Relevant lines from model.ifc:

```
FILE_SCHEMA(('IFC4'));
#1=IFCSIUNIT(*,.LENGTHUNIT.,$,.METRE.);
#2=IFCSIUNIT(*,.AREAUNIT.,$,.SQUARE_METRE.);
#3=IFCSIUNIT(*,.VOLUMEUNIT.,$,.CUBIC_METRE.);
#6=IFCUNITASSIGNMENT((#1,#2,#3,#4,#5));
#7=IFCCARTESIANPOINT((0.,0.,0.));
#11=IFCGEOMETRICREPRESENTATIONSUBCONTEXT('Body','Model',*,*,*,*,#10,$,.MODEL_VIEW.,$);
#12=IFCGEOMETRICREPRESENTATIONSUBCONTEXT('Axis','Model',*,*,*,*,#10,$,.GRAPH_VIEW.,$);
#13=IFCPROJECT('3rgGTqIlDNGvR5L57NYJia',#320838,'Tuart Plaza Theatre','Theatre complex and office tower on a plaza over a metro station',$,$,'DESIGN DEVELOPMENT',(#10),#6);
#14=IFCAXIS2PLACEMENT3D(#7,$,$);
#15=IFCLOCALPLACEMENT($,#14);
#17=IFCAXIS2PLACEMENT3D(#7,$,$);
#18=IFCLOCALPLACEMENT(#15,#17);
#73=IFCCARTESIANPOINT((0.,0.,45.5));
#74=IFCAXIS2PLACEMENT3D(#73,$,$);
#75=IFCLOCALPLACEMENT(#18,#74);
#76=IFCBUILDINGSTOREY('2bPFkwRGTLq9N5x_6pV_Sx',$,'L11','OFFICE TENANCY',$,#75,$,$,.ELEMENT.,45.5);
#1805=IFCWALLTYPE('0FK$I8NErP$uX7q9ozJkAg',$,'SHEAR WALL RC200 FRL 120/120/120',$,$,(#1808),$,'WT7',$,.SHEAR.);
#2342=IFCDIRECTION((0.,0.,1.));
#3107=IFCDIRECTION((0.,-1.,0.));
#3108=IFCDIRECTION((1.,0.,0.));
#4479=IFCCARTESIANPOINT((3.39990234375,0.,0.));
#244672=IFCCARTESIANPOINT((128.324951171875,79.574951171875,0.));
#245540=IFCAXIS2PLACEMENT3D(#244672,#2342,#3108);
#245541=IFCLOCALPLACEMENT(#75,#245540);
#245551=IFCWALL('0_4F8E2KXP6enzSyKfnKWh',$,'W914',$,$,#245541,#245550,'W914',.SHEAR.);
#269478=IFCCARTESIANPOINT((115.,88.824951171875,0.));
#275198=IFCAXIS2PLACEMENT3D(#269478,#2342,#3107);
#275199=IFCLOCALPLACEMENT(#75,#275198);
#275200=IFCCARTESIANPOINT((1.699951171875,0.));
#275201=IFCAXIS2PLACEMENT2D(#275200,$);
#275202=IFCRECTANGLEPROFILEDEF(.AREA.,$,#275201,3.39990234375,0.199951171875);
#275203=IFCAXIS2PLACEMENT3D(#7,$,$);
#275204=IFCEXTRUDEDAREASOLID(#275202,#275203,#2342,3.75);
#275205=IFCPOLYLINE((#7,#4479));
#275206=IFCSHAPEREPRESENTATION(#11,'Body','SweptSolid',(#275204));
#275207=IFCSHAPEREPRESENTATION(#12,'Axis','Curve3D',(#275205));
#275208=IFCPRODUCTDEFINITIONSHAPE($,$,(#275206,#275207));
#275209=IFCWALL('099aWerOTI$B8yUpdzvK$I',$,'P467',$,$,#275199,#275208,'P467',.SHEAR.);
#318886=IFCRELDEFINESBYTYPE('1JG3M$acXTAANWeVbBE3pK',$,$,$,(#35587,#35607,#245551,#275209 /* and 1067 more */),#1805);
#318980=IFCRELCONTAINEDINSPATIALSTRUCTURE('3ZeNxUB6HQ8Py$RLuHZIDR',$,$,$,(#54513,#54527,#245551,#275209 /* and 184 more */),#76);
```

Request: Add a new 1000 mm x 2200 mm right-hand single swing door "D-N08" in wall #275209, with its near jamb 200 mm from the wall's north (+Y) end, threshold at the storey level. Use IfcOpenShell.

```python
import numpy as np
import ifcopenshell
import ifcopenshell.api.feature
import ifcopenshell.api.geometry
import ifcopenshell.api.root
import ifcopenshell.api.spatial
import ifcopenshell.geom
import ifcopenshell.util.element
import ifcopenshell.util.placement
import ifcopenshell.util.representation
import ifcopenshell.util.shape
import ifcopenshell.util.unit

model = ifcopenshell.open("model.ifc")
unit_scale = ifcopenshell.util.unit.calculate_unit_scale(model)
settings = ifcopenshell.geom.settings()


def volume(element):
    """Net volume in cubic metres, openings subtracted."""
    shape = ifcopenshell.geom.create_shape(settings, element)
    return ifcopenshell.util.shape.get_volume(shape.geometry)


wall = model.by_guid("099aWerOTI$B8yUpdzvK$I")
storey = ifcopenshell.util.element.get_container(wall, ifc_class="IfcBuildingStorey")
context = ifcopenshell.util.representation.get_context(model, "Model", "Body", "MODEL_VIEW")
before = volume(wall)

width, height, from_end, sill = 1, 2.2, 0.2, 0.0  # metres

# The wall runs along its own X axis, and the end named is its -X end.
wall_shape = ifcopenshell.geom.create_shape(settings, wall)
x, y, z = ifcopenshell.util.shape.get_vertices(wall_shape.geometry).T
start = x.min() + from_end
face, thickness = float(y.min()), float(y.max() - y.min())
wall_matrix = ifcopenshell.util.placement.get_local_placement(wall.ObjectPlacement)
level = ifcopenshell.util.placement.get_local_placement(storey.ObjectPlacement)[2, 3]


def in_wall(x, y):
    """Placement at x, y metres in the wall's axes, at sill height."""
    matrix = wall_matrix.copy()
    matrix[:, 3] = wall_matrix @ np.array([x / unit_scale, y / unit_scale, 0.0, 1.0])
    matrix[2, 3] = level + sill / unit_scale
    return matrix


# Opening: a box that overshoots both wall faces by 50 mm.
opening = ifcopenshell.api.root.create_entity(model, ifc_class="IfcOpeningElement", predefined_type="OPENING")
box = ifcopenshell.api.geometry.add_wall_representation(
    model, context=context, length=width, height=height, thickness=thickness + 0.1
)
ifcopenshell.api.geometry.assign_representation(model, product=opening, representation=box)
ifcopenshell.api.geometry.edit_object_placement(model, product=opening, matrix=in_wall(start, face - 0.05), is_si=False)
ifcopenshell.api.feature.add_feature(model, feature=opening, element=wall)

door = ifcopenshell.api.root.create_entity(model, ifc_class="IfcDoor", name="D-N08", predefined_type="DOOR")
door.OverallWidth, door.OverallHeight = width / unit_scale, height / unit_scale
door.OperationType = "SINGLE_SWING_RIGHT"
body = ifcopenshell.api.geometry.add_door_representation(
    model,
    context=context,
    overall_width=door.OverallWidth,
    overall_height=door.OverallHeight,
    operation_type="SINGLE_SWING_RIGHT",
    lining_properties={"LiningDepth": thickness / unit_scale, "ThresholdDepth": thickness / unit_scale},
)
ifcopenshell.api.geometry.assign_representation(model, product=door, representation=body)
ifcopenshell.api.spatial.assign_container(model, products=[door], relating_structure=storey)
ifcopenshell.api.feature.add_filling(model, opening=opening, element=door)

# The lining spans the wall, so the door starts at the wall face.
ifcopenshell.api.geometry.edit_object_placement(model, product=door, matrix=in_wall(start, face), is_si=False)

after = volume(wall)

print(f"wall volume {before:.3f} -> {after:.3f} m3")

model.write("model-out.ifc")
```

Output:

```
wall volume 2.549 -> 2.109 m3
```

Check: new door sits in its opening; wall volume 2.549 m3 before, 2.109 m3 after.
